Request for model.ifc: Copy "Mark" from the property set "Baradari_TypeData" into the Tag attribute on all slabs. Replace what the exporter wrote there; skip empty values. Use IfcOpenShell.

First a look at what the model holds.

```python
import ifcopenshell
import ifcopenshell.util.element

model = ifcopenshell.open("model.ifc")
print(model.schema)
slabs = model.by_type("IfcSlab")
print(len(slabs), "slabs")
for e in slabs[:8]:
    source = ifcopenshell.util.element.get_pset(e, "Baradari_TypeData", "Mark")
    target = e.Tag
    print(e.id(), repr(source), repr(target), sep=" | ")
```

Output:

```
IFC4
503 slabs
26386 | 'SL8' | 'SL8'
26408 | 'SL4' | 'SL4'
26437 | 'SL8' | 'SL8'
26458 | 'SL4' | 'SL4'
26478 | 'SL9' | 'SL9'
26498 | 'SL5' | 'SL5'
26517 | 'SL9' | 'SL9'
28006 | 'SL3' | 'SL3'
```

```python
import ifcopenshell
import ifcopenshell.util.element

model = ifcopenshell.open("model.ifc")

count = 0
for e in model.by_type("IfcSlab"):
    value = ifcopenshell.util.element.get_pset(e, "Baradari_TypeData", "Mark")
    current = e.Tag
    if not value or not value.strip() or current == value:
        continue
    e.Tag = value
    count += 1

print(count, "slabs updated")

model.write("model_v2.ifc")
```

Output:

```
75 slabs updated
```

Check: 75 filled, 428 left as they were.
